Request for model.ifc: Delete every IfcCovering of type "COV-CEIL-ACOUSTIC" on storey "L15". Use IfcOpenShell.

First a look at what the model holds.

```python
import ifcopenshell
import ifcopenshell.util.element

model = ifcopenshell.open("model.ifc")
print(model.schema)
storey = next(s for s in model.by_type("IfcBuildingStorey") if s.Name == "L15")
coverings = [e for e in ifcopenshell.util.element.get_decomposition(storey) if e.is_a("IfcCovering")]
seen = {}
for e in coverings:
    element_type = ifcopenshell.util.element.get_type(e)
    name = element_type.Name if element_type not in (None, e) else None
    seen[name] = seen.get(name, 0) + 1
for name, count in sorted(seen.items(), key=str):
    print(count, "x", name)
```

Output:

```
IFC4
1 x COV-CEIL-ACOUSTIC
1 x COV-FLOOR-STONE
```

```python
import ifcopenshell
import ifcopenshell.api.root
import ifcopenshell.util.element

model = ifcopenshell.open("model.ifc")

storey = next(s for s in model.by_type("IfcBuildingStorey") if s.Name == "L15")
coverings = [e for e in ifcopenshell.util.element.get_decomposition(storey) if e.is_a("IfcCovering")]
targets = [e for e in coverings if (t := ifcopenshell.util.element.get_type(e)) not in (None, e) and t.Name == "COV-CEIL-ACOUSTIC"]

for e in targets:
    ifcopenshell.api.root.remove_product(model, product=e)
print(len(targets), "removed")

model.write("model-out.ifc")
```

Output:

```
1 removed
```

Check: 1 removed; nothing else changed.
